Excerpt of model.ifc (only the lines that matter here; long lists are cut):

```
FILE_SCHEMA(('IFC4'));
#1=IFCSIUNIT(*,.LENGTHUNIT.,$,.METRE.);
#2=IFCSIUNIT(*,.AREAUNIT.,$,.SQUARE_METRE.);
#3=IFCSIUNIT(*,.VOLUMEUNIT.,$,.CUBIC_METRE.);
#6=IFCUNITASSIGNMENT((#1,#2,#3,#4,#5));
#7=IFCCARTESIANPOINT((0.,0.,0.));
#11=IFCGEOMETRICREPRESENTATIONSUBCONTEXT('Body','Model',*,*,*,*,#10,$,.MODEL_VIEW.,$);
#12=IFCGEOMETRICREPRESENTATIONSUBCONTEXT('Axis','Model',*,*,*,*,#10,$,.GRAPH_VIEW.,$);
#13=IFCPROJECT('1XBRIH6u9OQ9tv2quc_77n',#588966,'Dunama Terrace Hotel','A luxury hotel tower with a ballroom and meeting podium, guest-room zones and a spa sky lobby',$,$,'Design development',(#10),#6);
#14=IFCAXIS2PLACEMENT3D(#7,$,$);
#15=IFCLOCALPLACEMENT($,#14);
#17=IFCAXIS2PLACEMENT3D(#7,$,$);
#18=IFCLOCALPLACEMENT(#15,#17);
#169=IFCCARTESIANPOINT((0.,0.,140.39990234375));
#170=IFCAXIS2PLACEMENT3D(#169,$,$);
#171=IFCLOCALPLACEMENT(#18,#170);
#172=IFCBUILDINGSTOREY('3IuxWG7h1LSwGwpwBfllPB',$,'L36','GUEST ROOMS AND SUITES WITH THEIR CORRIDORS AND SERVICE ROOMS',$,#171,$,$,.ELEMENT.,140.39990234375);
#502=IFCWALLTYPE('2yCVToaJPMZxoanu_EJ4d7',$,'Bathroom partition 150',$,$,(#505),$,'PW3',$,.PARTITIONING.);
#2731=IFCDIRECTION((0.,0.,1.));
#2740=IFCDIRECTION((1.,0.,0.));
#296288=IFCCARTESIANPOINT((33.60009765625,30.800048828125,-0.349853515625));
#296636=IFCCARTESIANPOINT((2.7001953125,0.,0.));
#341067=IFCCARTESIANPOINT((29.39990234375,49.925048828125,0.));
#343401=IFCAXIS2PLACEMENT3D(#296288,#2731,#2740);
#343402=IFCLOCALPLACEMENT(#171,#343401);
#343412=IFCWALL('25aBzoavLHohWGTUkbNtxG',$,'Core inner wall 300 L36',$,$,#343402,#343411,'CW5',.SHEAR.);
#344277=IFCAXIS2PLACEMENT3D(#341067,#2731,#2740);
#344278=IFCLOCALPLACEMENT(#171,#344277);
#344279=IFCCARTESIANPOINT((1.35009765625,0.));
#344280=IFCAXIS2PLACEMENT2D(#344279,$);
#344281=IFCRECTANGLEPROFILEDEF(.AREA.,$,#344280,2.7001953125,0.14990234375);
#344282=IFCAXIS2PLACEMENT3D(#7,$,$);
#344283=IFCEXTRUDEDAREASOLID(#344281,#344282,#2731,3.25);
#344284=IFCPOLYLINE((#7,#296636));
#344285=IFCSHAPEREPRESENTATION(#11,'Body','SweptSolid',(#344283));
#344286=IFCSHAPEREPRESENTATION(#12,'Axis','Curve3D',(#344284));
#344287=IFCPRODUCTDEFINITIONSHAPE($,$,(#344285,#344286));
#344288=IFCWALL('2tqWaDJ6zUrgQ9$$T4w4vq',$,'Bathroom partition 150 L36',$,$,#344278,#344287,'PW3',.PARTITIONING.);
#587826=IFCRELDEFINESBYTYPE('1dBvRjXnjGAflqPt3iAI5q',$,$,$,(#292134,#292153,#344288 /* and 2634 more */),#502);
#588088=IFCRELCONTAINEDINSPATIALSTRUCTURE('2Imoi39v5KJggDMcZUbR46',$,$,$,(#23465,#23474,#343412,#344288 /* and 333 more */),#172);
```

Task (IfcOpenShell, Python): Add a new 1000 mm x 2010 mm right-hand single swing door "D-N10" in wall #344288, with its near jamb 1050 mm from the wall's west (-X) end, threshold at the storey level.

```python
import numpy as np
import ifcopenshell
import ifcopenshell.api.feature
import ifcopenshell.api.geometry
import ifcopenshell.api.root
import ifcopenshell.api.spatial
import ifcopenshell.geom
import ifcopenshell.util.element
import ifcopenshell.util.placement
import ifcopenshell.util.representation
import ifcopenshell.util.shape
import ifcopenshell.util.unit

model = ifcopenshell.open("model.ifc")
unit_scale = ifcopenshell.util.unit.calculate_unit_scale(model)
settings = ifcopenshell.geom.settings()


def volume(element):
    """Net volume in cubic metres, openings subtracted."""
    shape = ifcopenshell.geom.create_shape(settings, element)
    return ifcopenshell.util.shape.get_volume(shape.geometry)


wall = model.by_id(344288)
storey = ifcopenshell.util.element.get_container(wall, ifc_class="IfcBuildingStorey")
context = ifcopenshell.util.representation.get_context(model, "Model", "Body", "MODEL_VIEW")
before = volume(wall)

width, height, from_end, sill = 1, 2.01, 1.05, 0.0  # metres

# The wall runs along its own X axis, and the end named is its -X end.
wall_shape = ifcopenshell.geom.create_shape(settings, wall)
x, y, z = ifcopenshell.util.shape.get_vertices(wall_shape.geometry).T
start = x.min() + from_end
face, thickness = float(y.min()), float(y.max() - y.min())
wall_matrix = ifcopenshell.util.placement.get_local_placement(wall.ObjectPlacement)
level = ifcopenshell.util.placement.get_local_placement(storey.ObjectPlacement)[2, 3]


def in_wall(x, y):
    """Placement at x, y metres in the wall's axes, at sill height."""
    matrix = wall_matrix.copy()
    matrix[:, 3] = wall_matrix @ np.array([x / unit_scale, y / unit_scale, 0.0, 1.0])
    matrix[2, 3] = level + sill / unit_scale
    return matrix


# Opening: a box that overshoots both wall faces by 50 mm.
opening = ifcopenshell.api.root.create_entity(model, ifc_class="IfcOpeningElement", predefined_type="OPENING")
box = ifcopenshell.api.geometry.add_wall_representation(
    model, context=context, length=width, height=height, thickness=thickness + 0.1
)
ifcopenshell.api.geometry.assign_representation(model, product=opening, representation=box)
ifcopenshell.api.geometry.edit_object_placement(model, product=opening, matrix=in_wall(start, face - 0.05), is_si=False)
ifcopenshell.api.feature.add_feature(model, feature=opening, element=wall)

door = ifcopenshell.api.root.create_entity(model, ifc_class="IfcDoor", name="D-N10", predefined_type="DOOR")
door.OverallWidth, door.OverallHeight = width / unit_scale, height / unit_scale
door.OperationType = "SINGLE_SWING_RIGHT"
body = ifcopenshell.api.geometry.add_door_representation(
    model,
    context=context,
    overall_width=door.OverallWidth,
    overall_height=door.OverallHeight,
    operation_type="SINGLE_SWING_RIGHT",
    lining_properties={"LiningDepth": thickness / unit_scale, "ThresholdDepth": thickness / unit_scale},
)
ifcopenshell.api.geometry.assign_representation(model, product=door, representation=body)
ifcopenshell.api.spatial.assign_container(model, products=[door], relating_structure=storey)
ifcopenshell.api.feature.add_filling(model, opening=opening, element=door)

# The lining spans the wall, so the door starts at the wall face.
ifcopenshell.api.geometry.edit_object_placement(model, product=door, matrix=in_wall(start, face), is_si=False)

after = volume(wall)

print(f"wall volume {before:.3f} -> {after:.3f} m3")

model.write("model_v2.ifc")
```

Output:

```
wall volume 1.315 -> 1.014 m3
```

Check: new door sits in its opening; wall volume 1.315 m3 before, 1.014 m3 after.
